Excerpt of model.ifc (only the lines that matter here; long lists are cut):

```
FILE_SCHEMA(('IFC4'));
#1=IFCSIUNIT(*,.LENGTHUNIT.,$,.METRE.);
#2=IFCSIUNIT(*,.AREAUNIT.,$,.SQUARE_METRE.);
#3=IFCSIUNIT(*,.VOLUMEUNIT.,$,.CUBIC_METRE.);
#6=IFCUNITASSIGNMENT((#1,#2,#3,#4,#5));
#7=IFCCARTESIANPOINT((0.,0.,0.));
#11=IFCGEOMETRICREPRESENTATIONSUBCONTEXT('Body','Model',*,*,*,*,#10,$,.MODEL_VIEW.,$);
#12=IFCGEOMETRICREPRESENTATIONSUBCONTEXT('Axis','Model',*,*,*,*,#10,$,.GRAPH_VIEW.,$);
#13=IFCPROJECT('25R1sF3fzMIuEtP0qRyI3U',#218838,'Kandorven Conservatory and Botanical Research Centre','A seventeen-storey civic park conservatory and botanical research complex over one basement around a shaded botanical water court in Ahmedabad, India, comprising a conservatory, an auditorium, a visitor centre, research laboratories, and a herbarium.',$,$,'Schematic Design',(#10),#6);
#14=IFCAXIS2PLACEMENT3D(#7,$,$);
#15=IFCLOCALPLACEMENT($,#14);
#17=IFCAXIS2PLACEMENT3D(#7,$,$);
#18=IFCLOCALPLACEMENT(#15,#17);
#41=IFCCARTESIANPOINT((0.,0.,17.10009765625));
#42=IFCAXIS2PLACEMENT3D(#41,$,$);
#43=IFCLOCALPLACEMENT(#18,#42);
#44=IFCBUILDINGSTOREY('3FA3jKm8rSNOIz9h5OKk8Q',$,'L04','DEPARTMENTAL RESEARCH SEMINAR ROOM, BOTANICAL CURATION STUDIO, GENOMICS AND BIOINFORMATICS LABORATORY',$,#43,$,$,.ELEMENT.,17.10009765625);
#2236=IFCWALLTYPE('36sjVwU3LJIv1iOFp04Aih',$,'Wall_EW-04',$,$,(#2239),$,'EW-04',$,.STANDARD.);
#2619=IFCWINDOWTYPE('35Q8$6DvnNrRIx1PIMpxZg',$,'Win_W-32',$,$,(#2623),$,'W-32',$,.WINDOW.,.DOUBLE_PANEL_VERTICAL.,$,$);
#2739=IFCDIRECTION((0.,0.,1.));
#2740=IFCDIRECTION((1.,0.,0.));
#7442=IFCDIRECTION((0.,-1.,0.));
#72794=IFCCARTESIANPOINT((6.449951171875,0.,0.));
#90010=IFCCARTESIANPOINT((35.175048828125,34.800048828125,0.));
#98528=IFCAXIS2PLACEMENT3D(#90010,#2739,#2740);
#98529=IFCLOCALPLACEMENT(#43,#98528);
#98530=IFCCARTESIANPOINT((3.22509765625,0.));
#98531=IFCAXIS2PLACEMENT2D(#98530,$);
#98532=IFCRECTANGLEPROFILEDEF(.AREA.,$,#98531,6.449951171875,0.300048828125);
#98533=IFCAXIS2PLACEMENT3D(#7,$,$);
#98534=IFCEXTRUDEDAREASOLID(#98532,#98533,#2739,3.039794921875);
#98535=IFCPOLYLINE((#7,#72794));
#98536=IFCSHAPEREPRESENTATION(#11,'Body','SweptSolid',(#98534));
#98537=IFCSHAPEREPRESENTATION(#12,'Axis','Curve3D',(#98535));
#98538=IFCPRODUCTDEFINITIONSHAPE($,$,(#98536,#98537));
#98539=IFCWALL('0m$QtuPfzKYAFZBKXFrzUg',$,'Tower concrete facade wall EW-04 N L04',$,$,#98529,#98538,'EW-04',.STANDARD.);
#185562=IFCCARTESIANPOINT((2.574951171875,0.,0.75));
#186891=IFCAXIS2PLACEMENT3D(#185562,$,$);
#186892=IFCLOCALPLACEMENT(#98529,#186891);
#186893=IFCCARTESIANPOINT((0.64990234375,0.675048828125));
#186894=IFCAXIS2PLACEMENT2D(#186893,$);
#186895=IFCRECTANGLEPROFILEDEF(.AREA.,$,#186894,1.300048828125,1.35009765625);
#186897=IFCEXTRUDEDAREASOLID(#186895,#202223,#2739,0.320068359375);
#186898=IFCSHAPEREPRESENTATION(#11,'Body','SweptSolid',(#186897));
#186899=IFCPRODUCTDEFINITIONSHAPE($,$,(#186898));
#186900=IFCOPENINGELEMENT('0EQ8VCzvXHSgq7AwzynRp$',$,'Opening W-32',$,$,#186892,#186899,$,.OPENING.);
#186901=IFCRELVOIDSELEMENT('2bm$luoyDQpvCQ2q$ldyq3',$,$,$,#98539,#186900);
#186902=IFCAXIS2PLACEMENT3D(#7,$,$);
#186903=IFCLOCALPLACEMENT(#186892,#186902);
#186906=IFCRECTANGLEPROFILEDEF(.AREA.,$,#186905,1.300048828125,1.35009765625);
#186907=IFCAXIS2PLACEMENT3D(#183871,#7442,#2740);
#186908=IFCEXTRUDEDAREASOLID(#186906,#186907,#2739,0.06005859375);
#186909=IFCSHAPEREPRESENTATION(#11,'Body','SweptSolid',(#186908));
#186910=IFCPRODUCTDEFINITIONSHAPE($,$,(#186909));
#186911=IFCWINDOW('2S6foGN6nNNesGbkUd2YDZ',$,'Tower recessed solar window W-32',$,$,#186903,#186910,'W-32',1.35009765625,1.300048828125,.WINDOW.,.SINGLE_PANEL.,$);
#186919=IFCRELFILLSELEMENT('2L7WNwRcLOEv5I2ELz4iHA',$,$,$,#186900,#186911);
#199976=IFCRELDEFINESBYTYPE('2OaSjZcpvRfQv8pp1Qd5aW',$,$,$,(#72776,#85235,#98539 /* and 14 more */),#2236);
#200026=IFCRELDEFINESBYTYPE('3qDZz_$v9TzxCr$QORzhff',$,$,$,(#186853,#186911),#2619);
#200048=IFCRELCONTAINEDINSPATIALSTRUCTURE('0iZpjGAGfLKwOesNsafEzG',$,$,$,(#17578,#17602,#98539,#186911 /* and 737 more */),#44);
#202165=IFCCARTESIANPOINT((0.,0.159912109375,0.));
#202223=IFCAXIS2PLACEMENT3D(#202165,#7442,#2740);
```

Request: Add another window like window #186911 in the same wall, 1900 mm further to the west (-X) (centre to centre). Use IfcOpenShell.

```python
import ifcopenshell
import ifcopenshell.api.feature
import ifcopenshell.api.geometry
import ifcopenshell.api.root
import ifcopenshell.geom
import ifcopenshell.util.element
import ifcopenshell.util.placement
import ifcopenshell.util.shape

model = ifcopenshell.open("model.ifc")
settings = ifcopenshell.geom.settings()


def volume(element):
    """Net volume in cubic metres, openings subtracted."""
    shape = ifcopenshell.geom.create_shape(settings, element)
    return ifcopenshell.util.shape.get_volume(shape.geometry)


window = model.by_guid("2S6foGN6nNNesGbkUd2YDZ")
opening = window.FillsVoids[0].RelatingOpeningElement
wall = opening.VoidsElements[0].RelatingBuildingElement
before = volume(wall)
shift = ifcopenshell.util.placement.get_local_placement(wall.ObjectPlacement)[:3, 0] * -1.9

# copy_class copies the void relationship, type, container and properties, but no geometry.
new_opening = ifcopenshell.api.root.copy_class(model, product=opening)
new_opening.Representation = ifcopenshell.util.element.copy_deep(
    model, opening.Representation, exclude=["IfcGeometricRepresentationContext", "IfcRepresentationMap"]
)
new_window = ifcopenshell.api.root.copy_class(model, product=window)
new_window.Representation = ifcopenshell.util.element.copy_deep(
    model, window.Representation, exclude=["IfcGeometricRepresentationContext", "IfcRepresentationMap"]
)
new_window.Tag = None
ifcopenshell.api.feature.add_filling(model, opening=new_opening, element=new_window)

for old, new in ((opening, new_opening), (window, new_window)):
    matrix = ifcopenshell.util.placement.get_local_placement(old.ObjectPlacement)
    matrix[:3, 3] += shift
    ifcopenshell.api.geometry.edit_object_placement(model, product=new, matrix=matrix, is_si=False)

after = volume(wall)

print(f"wall volume {before:.3f} -> {after:.3f} m3")

model.write("model_v2.ifc")
```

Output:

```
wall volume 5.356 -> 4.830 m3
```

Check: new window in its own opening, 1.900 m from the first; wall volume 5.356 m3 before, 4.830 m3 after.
